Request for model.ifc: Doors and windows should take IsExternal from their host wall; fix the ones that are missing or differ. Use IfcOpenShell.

First a look at what the model holds.

```python
import ifcopenshell
import ifcopenshell.util.element

model = ifcopenshell.open("model.ifc")
print(model.schema)
seen = {}
for e in model.by_type("IfcDoor") + model.by_type("IfcWindow"):
    if not e.FillsVoids:
        continue
    host = e.FillsVoids[0].RelatingOpeningElement.VoidsElements[0].RelatingBuildingElement
    own = ifcopenshell.util.element.get_pset(e, f"Pset_{e.is_a()[3:].removesuffix('StandardCase')}Common", "IsExternal")
    wall = ifcopenshell.util.element.get_pset(host, "Pset_WallCommon", "IsExternal")
    seen[e.is_a(), own, wall] = seen.get((e.is_a(), own, wall), 0) + 1
for (cls, own, wall), count in sorted(seen.items(), key=str):
    print(count, cls, "IsExternal:", own, "| host wall:", wall)
```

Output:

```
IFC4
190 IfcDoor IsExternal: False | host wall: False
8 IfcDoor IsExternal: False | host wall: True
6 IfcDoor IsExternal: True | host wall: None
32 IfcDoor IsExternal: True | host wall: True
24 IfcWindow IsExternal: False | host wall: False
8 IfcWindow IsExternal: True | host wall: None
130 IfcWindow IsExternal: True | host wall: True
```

```python
import ifcopenshell
import ifcopenshell.api.pset
import ifcopenshell.util.element

model = ifcopenshell.open("model.ifc")

count = 0
for ifc_class, pset_name in (("IfcDoor", "Pset_DoorCommon"), ("IfcWindow", "Pset_WindowCommon")):
    for e in model.by_type(ifc_class):
        if not e.FillsVoids:
            continue
        host = e.FillsVoids[0].RelatingOpeningElement.VoidsElements[0].RelatingBuildingElement
        external = ifcopenshell.util.element.get_pset(host, "Pset_WallCommon", "IsExternal")
        if external is None or ifcopenshell.util.element.get_pset(e, pset_name, "IsExternal") == external:
            continue
        pset = ifcopenshell.api.pset.add_pset(model, product=e, name=pset_name)
        ifcopenshell.api.pset.edit_pset(model, pset=pset, properties={"IsExternal": external})
        count += 1

print(count, "updated")

model.write("model-out.ifc")
```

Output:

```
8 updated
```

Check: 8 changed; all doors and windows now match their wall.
